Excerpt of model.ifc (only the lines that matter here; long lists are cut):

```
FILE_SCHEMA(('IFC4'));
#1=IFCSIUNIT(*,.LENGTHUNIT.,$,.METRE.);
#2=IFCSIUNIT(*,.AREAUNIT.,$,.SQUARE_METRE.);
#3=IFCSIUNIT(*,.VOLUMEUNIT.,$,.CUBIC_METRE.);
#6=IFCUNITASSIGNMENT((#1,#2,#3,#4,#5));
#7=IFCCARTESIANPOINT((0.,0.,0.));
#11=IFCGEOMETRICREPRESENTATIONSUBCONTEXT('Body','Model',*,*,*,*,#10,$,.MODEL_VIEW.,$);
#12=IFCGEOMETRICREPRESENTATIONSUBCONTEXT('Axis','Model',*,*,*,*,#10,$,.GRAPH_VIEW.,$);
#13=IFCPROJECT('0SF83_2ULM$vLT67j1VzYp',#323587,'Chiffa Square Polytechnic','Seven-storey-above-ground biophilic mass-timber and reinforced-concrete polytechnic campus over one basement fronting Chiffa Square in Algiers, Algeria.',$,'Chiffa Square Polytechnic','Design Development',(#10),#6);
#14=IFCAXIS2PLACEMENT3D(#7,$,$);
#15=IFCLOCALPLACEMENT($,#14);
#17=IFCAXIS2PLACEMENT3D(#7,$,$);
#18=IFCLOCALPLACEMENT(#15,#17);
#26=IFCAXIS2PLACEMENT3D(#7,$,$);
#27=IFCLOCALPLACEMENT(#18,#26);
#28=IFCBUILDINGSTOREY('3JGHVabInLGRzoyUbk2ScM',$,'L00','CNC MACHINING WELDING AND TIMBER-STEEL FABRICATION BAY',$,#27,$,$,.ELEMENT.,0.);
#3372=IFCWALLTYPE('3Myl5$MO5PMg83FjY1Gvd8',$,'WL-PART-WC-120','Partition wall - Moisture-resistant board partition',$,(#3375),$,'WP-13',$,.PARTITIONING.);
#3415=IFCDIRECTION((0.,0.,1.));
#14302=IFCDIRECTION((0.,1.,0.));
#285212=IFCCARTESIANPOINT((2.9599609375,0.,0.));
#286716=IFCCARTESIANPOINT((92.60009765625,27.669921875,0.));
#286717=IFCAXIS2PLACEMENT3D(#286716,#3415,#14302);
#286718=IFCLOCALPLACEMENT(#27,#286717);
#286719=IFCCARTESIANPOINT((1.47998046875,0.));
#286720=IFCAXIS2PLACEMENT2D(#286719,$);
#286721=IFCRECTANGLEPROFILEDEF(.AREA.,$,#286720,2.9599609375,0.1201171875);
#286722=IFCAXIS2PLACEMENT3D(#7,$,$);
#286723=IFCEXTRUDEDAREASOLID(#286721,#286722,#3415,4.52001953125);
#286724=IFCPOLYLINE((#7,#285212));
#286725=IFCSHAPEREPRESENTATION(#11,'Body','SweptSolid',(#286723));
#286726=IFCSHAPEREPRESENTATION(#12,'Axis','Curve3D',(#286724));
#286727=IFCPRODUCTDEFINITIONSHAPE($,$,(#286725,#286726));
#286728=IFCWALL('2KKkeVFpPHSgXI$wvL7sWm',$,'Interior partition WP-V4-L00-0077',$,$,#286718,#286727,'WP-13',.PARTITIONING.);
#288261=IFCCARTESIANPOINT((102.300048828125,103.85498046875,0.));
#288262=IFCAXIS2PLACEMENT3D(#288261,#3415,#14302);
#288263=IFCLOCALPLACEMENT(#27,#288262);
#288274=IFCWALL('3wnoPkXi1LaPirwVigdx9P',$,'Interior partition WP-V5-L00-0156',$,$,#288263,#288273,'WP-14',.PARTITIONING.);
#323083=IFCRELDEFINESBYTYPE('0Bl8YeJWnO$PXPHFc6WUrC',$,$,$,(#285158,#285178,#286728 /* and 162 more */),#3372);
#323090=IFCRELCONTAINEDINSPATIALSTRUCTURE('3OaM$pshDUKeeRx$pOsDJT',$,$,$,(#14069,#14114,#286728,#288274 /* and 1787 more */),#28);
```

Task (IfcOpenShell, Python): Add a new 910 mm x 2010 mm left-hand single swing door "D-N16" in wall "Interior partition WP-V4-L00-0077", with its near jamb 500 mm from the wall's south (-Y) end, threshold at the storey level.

```python
import numpy as np
import ifcopenshell
import ifcopenshell.api.feature
import ifcopenshell.api.geometry
import ifcopenshell.api.root
import ifcopenshell.api.spatial
import ifcopenshell.geom
import ifcopenshell.util.element
import ifcopenshell.util.placement
import ifcopenshell.util.representation
import ifcopenshell.util.shape
import ifcopenshell.util.unit

model = ifcopenshell.open("model.ifc")
unit_scale = ifcopenshell.util.unit.calculate_unit_scale(model)
settings = ifcopenshell.geom.settings()


def volume(element):
    """Net volume in cubic metres, openings subtracted."""
    shape = ifcopenshell.geom.create_shape(settings, element)
    return ifcopenshell.util.shape.get_volume(shape.geometry)


wall = model.by_guid("2KKkeVFpPHSgXI$wvL7sWm")
storey = ifcopenshell.util.element.get_container(wall, ifc_class="IfcBuildingStorey")
context = ifcopenshell.util.representation.get_context(model, "Model", "Body", "MODEL_VIEW")
before = volume(wall)

width, height, from_end, sill = 0.91, 2.01, 0.5, 0.0  # metres

# The wall runs along its own X axis, and the end named is its -X end.
wall_shape = ifcopenshell.geom.create_shape(settings, wall)
x, y, z = ifcopenshell.util.shape.get_vertices(wall_shape.geometry).T
start = x.min() + from_end
face, thickness = float(y.min()), float(y.max() - y.min())
wall_matrix = ifcopenshell.util.placement.get_local_placement(wall.ObjectPlacement)
level = ifcopenshell.util.placement.get_local_placement(storey.ObjectPlacement)[2, 3]


def in_wall(x, y):
    """Placement at x, y metres in the wall's axes, at sill height."""
    matrix = wall_matrix.copy()
    matrix[:, 3] = wall_matrix @ np.array([x / unit_scale, y / unit_scale, 0.0, 1.0])
    matrix[2, 3] = level + sill / unit_scale
    return matrix


# Opening: a box that overshoots both wall faces by 50 mm.
opening = ifcopenshell.api.root.create_entity(model, ifc_class="IfcOpeningElement", predefined_type="OPENING")
box = ifcopenshell.api.geometry.add_wall_representation(
    model, context=context, length=width, height=height, thickness=thickness + 0.1
)
ifcopenshell.api.geometry.assign_representation(model, product=opening, representation=box)
ifcopenshell.api.geometry.edit_object_placement(model, product=opening, matrix=in_wall(start, face - 0.05), is_si=False)
ifcopenshell.api.feature.add_feature(model, feature=opening, element=wall)

door = ifcopenshell.api.root.create_entity(model, ifc_class="IfcDoor", name="D-N16", predefined_type="DOOR")
door.OverallWidth, door.OverallHeight = width / unit_scale, height / unit_scale
door.OperationType = "SINGLE_SWING_LEFT"
body = ifcopenshell.api.geometry.add_door_representation(
    model,
    context=context,
    overall_width=door.OverallWidth,
    overall_height=door.OverallHeight,
    operation_type="SINGLE_SWING_LEFT",
    lining_properties={"LiningDepth": thickness / unit_scale, "ThresholdDepth": thickness / unit_scale},
)
ifcopenshell.api.geometry.assign_representation(model, product=door, representation=body)
ifcopenshell.api.spatial.assign_container(model, products=[door], relating_structure=storey)
ifcopenshell.api.feature.add_filling(model, opening=opening, element=door)

# The lining spans the wall, so the door starts at the wall face.
ifcopenshell.api.geometry.edit_object_placement(model, product=door, matrix=in_wall(start, face), is_si=False)

after = volume(wall)

print(f"wall volume {before:.3f} -> {after:.3f} m3")

model.write("model_updated.ifc")
```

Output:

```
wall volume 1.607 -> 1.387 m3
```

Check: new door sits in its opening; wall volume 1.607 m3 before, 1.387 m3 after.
